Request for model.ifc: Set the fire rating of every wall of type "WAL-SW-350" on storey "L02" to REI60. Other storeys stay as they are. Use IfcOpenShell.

First a look at what the model holds.

```python
import ifcopenshell
import ifcopenshell.util.element

model = ifcopenshell.open("model.ifc")
print(model.schema)
storey = next(s for s in model.by_type("IfcBuildingStorey") if s.Name == "L02")
walls = [e for e in ifcopenshell.util.element.get_decomposition(storey) if e.is_a("IfcWall")]
seen = {}
for e in walls:
    element_type = ifcopenshell.util.element.get_type(e)
    key = (element_type.Name if element_type != e and element_type else None, ifcopenshell.util.element.get_pset(e, "Pset_WallCommon", "FireRating"))
    seen[key] = seen.get(key, 0) + 1
for (name, value), count in sorted(seen.items(), key=str):
    print(count, "x", name, "|", value)
```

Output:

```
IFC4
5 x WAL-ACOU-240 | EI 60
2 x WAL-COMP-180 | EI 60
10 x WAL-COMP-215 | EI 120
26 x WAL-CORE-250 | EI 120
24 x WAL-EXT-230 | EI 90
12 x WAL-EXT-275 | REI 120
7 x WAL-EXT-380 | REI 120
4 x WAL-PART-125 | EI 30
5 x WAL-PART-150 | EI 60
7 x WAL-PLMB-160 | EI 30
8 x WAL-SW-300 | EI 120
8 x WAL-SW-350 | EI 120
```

```python
import ifcopenshell
import ifcopenshell.api.pset
import ifcopenshell.util.element

model = ifcopenshell.open("model.ifc")

storey = next(s for s in model.by_type("IfcBuildingStorey") if s.Name == "L02")
walls = [e for e in ifcopenshell.util.element.get_decomposition(storey) if e.is_a("IfcWall")]

count = 0
for e in walls:
    element_type = ifcopenshell.util.element.get_type(e)
    if element_type in (None, e) or element_type.Name != "WAL-SW-350":
        continue
    # add_pset returns the element's existing set when there is one.
    pset = ifcopenshell.api.pset.add_pset(model, product=e, name="Pset_WallCommon")
    ifcopenshell.api.pset.edit_pset(model, pset=pset, properties={"FireRating": "REI60"})
    count += 1

print(count, "walls updated")

model.write("model_edited.ifc")
```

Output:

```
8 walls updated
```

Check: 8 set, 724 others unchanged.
